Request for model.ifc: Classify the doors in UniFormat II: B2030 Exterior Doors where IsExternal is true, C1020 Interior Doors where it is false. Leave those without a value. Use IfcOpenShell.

First a look at what the model holds.

```python
import ifcopenshell
import ifcopenshell.util.element

model = ifcopenshell.open("model.ifc")
print(model.schema)
print("classifications:", [c.Name for c in model.by_type("IfcClassification")])
values = [ifcopenshell.util.element.get_pset(e, "Pset_DoorCommon", "IsExternal") for e in model.by_type("IfcDoor")]
for value in (True, False, None):
    print("IsExternal", value, values.count(value))
```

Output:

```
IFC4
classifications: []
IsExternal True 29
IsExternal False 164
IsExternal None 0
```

```python
import ifcopenshell
import ifcopenshell.api.classification
import ifcopenshell.util.element

model = ifcopenshell.open("model.ifc")

system = ifcopenshell.api.classification.add_classification(model, classification="UniFormat II")

doors = model.by_type("IfcDoor")
external = {e: ifcopenshell.util.element.get_pset(e, "Pset_DoorCommon", "IsExternal") for e in doors}
for flag, code, name in ((True, "B2030", "Exterior Doors"), (False, "C1020", "Interior Doors")):
    products = [e for e in doors if external[e] is flag]
    ifcopenshell.api.classification.add_reference(
        model, products=products, classification=system, identification=code, name=name
    )
    print(code, len(products))

model.write("model_edited.ifc")
```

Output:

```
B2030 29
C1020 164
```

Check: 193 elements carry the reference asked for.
